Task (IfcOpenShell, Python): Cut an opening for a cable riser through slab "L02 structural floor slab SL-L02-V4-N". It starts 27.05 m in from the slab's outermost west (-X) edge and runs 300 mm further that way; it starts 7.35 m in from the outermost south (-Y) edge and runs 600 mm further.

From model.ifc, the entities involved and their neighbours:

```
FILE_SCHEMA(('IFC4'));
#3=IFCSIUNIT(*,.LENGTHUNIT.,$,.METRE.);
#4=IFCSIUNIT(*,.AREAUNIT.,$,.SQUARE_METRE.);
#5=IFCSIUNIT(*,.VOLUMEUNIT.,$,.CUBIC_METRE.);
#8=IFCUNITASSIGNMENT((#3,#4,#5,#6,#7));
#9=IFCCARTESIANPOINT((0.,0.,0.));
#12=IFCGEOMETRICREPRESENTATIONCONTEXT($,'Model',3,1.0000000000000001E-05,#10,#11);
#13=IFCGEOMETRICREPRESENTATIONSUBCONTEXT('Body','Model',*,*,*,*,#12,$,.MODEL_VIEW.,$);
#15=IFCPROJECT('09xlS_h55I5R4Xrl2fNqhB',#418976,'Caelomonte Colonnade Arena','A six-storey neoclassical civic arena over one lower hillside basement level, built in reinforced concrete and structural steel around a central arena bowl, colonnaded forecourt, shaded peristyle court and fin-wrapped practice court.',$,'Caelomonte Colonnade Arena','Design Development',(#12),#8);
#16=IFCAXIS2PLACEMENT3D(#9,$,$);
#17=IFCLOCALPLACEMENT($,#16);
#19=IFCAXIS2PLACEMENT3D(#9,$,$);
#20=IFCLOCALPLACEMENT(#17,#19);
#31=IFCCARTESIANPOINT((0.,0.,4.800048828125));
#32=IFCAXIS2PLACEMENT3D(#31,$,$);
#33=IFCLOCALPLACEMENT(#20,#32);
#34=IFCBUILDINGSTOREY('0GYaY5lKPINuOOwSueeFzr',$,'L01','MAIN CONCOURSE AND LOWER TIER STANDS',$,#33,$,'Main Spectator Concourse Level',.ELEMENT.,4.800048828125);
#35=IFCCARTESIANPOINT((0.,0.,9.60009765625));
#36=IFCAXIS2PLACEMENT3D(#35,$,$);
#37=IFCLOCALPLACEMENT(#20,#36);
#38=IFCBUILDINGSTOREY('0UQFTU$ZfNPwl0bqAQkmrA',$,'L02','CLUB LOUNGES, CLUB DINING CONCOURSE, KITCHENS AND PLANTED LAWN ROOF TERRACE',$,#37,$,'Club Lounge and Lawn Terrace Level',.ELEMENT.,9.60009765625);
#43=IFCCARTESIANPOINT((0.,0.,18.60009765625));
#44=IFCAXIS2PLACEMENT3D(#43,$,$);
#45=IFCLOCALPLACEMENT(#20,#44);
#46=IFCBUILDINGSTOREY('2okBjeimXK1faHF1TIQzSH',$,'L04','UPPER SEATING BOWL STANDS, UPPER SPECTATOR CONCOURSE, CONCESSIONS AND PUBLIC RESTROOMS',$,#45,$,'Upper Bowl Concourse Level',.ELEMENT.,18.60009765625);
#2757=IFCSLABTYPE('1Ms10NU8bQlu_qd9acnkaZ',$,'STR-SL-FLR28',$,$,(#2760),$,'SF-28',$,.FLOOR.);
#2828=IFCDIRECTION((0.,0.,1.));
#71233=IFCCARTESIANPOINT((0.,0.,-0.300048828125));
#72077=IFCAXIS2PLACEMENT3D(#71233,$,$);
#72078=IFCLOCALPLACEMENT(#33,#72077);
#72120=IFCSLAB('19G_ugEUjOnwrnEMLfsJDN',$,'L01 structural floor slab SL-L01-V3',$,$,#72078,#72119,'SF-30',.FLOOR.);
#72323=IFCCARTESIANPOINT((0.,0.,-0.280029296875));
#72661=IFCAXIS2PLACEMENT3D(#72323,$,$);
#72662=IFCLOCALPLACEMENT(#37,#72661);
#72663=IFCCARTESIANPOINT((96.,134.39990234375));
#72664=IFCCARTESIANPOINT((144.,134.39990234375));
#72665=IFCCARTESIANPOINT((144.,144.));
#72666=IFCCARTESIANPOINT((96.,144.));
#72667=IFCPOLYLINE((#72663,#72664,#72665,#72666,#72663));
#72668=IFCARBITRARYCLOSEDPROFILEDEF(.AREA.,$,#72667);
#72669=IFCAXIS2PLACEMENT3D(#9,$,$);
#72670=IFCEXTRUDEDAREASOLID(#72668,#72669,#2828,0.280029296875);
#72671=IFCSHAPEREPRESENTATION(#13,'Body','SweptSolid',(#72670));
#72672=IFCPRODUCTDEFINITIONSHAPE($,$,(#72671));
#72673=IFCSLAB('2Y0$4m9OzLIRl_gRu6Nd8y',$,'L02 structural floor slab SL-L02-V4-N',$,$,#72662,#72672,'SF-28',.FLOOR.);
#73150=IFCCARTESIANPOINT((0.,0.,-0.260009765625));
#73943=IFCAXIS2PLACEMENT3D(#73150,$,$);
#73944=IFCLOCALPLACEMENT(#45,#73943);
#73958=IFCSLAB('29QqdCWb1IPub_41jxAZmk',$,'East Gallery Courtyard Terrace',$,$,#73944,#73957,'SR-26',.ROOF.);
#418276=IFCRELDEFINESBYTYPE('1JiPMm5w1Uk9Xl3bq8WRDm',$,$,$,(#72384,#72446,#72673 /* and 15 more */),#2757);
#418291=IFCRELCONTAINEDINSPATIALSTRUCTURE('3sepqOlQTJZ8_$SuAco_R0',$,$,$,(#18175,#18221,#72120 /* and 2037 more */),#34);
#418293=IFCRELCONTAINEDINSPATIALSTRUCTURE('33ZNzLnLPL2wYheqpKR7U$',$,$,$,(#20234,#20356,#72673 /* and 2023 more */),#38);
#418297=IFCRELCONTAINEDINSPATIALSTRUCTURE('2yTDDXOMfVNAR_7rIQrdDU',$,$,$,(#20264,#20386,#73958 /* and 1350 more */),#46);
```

```python
import numpy as np
import ifcopenshell
import ifcopenshell.api.feature
import ifcopenshell.api.geometry
import ifcopenshell.api.root
import ifcopenshell.geom
import ifcopenshell.util.placement
import ifcopenshell.util.representation
import ifcopenshell.util.shape
import ifcopenshell.util.unit

model = ifcopenshell.open("model.ifc")
unit_scale = ifcopenshell.util.unit.calculate_unit_scale(model)
settings = ifcopenshell.geom.settings()


def volume(element):
    """Net volume in cubic metres, openings subtracted."""
    shape = ifcopenshell.geom.create_shape(settings, element)
    return ifcopenshell.util.shape.get_volume(shape.geometry)


slab = model.by_guid("2Y0$4m9OzLIRl_gRu6Nd8y")
before = volume(slab)

# Extent in the slab's own axes, in metres. The edges named are its -X and -Y sides.
slab_shape = ifcopenshell.geom.create_shape(settings, slab)
vertices = ifcopenshell.util.shape.get_vertices(slab_shape.geometry)
x_min, y_min, bottom = vertices.min(axis=0)
top = vertices[:, 2].max()

opening = ifcopenshell.api.root.create_entity(model, ifc_class="IfcOpeningElement", name="Cable riser opening", predefined_type="OPENING")
context = ifcopenshell.util.representation.get_context(model, "Model", "Body", "MODEL_VIEW")
width, depth = 0.3, 0.6
outline = [(0.0, 0.0), (width, 0.0), (width, depth), (0.0, depth), (0.0, 0.0)]
# Overshoot both faces by 50 mm so the cut is clean.
shape = ifcopenshell.api.geometry.add_slab_representation(
    model, context=context, depth=top - bottom + 0.1, polyline=outline
)
ifcopenshell.api.geometry.assign_representation(model, product=opening, representation=shape)

matrix = ifcopenshell.util.placement.get_local_placement(slab.ObjectPlacement)
matrix[:, 3] = matrix @ np.append(np.array([x_min + 27.05, y_min + 7.35, bottom - 0.05]) / unit_scale, 1.0)
ifcopenshell.api.geometry.edit_object_placement(model, product=opening, matrix=matrix, is_si=False)
ifcopenshell.api.feature.add_feature(model, feature=opening, element=slab)

after = volume(slab)

print(f"slab volume {before:.3f} -> {after:.3f} m3")

model.write("model_rev.ifc")
```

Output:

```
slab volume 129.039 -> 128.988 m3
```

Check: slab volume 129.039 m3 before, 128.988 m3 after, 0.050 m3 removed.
